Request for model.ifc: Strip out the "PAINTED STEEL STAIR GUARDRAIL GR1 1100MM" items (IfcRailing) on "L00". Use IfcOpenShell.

First a look at what the model holds.

```python
import ifcopenshell
import ifcopenshell.util.element

model = ifcopenshell.open("model.ifc")
print(model.schema)
storey = next(s for s in model.by_type("IfcBuildingStorey") if s.Name == "L00")
railings = [e for e in ifcopenshell.util.element.get_decomposition(storey) if e.is_a("IfcRailing")]
seen = {}
for e in railings:
    element_type = ifcopenshell.util.element.get_type(e)
    name = element_type.Name if element_type not in (None, e) else None
    seen[name] = seen.get(name, 0) + 1
for name, count in sorted(seen.items(), key=str):
    print(count, "x", name)
```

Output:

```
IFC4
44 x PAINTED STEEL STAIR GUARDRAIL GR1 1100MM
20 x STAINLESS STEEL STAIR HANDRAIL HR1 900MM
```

```python
import ifcopenshell
import ifcopenshell.api.root
import ifcopenshell.util.element

model = ifcopenshell.open("model.ifc")

storey = next(s for s in model.by_type("IfcBuildingStorey") if s.Name == "L00")
railings = [e for e in ifcopenshell.util.element.get_decomposition(storey) if e.is_a("IfcRailing")]
targets = [e for e in railings if (t := ifcopenshell.util.element.get_type(e)) not in (None, e) and t.Name == "PAINTED STEEL STAIR GUARDRAIL GR1 1100MM"]

for e in targets:
    ifcopenshell.api.root.remove_product(model, product=e)
print(len(targets), "removed")

model.write("model_rev.ifc")
```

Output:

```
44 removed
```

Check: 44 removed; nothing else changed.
